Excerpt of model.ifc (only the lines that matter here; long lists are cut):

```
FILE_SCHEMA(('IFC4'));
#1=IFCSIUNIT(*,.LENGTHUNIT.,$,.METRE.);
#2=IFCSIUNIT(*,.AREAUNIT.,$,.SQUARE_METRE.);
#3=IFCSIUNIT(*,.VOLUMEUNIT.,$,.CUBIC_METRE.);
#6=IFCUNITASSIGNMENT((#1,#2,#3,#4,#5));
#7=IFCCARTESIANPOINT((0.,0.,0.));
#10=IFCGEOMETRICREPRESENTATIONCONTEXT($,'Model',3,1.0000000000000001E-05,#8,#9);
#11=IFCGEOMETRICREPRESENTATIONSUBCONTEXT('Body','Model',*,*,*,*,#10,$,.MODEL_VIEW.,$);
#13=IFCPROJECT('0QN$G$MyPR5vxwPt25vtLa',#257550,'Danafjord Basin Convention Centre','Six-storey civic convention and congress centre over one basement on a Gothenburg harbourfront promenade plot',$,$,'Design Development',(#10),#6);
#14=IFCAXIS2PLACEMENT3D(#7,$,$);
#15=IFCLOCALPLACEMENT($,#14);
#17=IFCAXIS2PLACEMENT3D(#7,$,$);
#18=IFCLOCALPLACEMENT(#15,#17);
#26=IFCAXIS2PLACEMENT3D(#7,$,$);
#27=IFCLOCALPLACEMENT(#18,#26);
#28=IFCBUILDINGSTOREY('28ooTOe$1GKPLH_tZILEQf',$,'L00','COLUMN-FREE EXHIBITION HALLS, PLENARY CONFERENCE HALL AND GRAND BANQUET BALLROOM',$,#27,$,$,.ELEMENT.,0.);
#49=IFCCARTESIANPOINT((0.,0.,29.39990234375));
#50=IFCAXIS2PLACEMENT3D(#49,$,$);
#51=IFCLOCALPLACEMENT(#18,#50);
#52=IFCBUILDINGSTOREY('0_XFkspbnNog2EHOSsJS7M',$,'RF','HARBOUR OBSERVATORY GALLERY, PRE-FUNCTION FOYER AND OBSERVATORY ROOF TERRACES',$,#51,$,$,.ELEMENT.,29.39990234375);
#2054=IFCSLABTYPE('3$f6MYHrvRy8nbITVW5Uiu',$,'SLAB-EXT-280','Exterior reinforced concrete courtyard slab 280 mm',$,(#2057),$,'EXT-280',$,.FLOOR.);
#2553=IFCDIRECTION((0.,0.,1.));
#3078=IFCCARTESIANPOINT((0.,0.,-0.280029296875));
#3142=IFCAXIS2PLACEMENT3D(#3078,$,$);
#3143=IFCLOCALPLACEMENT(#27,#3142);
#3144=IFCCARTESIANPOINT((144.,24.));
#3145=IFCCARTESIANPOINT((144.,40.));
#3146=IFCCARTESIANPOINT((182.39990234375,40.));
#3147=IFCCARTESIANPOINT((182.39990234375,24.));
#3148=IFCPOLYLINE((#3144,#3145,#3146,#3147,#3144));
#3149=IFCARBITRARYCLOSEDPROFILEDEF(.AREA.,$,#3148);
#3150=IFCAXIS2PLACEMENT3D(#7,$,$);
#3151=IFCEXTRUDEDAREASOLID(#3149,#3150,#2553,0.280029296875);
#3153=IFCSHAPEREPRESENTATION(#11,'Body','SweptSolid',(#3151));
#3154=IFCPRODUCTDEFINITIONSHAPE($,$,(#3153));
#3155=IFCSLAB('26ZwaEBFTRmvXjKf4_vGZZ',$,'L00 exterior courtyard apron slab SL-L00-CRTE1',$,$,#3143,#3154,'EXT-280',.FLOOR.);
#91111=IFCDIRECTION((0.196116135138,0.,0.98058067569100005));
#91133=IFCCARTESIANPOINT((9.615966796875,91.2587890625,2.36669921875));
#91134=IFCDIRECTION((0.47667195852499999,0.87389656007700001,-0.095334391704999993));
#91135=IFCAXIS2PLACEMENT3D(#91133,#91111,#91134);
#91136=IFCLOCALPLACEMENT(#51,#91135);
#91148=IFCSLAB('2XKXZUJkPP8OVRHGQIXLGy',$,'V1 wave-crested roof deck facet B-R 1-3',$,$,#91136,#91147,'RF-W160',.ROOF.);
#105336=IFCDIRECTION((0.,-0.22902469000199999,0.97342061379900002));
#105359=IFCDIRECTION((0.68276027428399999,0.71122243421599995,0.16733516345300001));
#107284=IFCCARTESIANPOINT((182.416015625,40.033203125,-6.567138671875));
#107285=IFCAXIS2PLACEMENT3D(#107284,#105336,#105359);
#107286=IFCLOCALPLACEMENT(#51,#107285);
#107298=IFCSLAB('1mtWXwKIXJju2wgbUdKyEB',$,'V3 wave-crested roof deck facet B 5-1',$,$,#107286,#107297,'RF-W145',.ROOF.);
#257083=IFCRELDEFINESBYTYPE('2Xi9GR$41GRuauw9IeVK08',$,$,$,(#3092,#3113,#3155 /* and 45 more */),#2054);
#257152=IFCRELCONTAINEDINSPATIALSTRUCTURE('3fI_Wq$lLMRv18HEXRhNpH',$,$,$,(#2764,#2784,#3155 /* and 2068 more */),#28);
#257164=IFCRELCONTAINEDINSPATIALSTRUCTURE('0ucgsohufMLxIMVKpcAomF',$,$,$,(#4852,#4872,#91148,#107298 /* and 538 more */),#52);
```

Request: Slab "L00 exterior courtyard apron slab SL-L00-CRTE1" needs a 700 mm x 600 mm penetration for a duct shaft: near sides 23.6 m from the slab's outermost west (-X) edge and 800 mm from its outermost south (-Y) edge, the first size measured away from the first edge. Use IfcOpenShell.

```python
import numpy as np
import ifcopenshell
import ifcopenshell.api.feature
import ifcopenshell.api.geometry
import ifcopenshell.api.root
import ifcopenshell.geom
import ifcopenshell.util.placement
import ifcopenshell.util.representation
import ifcopenshell.util.shape
import ifcopenshell.util.unit

model = ifcopenshell.open("model.ifc")
unit_scale = ifcopenshell.util.unit.calculate_unit_scale(model)
settings = ifcopenshell.geom.settings()


def volume(element):
    """Net volume in cubic metres, openings subtracted."""
    shape = ifcopenshell.geom.create_shape(settings, element)
    return ifcopenshell.util.shape.get_volume(shape.geometry)


slab = model.by_id(3155)
before = volume(slab)

# Extent in the slab's own axes, in metres. The edges named are its -X and -Y sides.
slab_shape = ifcopenshell.geom.create_shape(settings, slab)
vertices = ifcopenshell.util.shape.get_vertices(slab_shape.geometry)
x_min, y_min, bottom = vertices.min(axis=0)
top = vertices[:, 2].max()

opening = ifcopenshell.api.root.create_entity(model, ifc_class="IfcOpeningElement", name="Duct shaft opening", predefined_type="OPENING")
context = ifcopenshell.util.representation.get_context(model, "Model", "Body", "MODEL_VIEW")
width, depth = 0.7, 0.6
outline = [(0.0, 0.0), (width, 0.0), (width, depth), (0.0, depth), (0.0, 0.0)]
# Overshoot both faces by 50 mm so the cut is clean.
shape = ifcopenshell.api.geometry.add_slab_representation(
    model, context=context, depth=top - bottom + 0.1, polyline=outline
)
ifcopenshell.api.geometry.assign_representation(model, product=opening, representation=shape)

matrix = ifcopenshell.util.placement.get_local_placement(slab.ObjectPlacement)
matrix[:, 3] = matrix @ np.append(np.array([x_min + 23.6, y_min + 0.8, bottom - 0.05]) / unit_scale, 1.0)
ifcopenshell.api.geometry.edit_object_placement(model, product=opening, matrix=matrix, is_si=False)
ifcopenshell.api.feature.add_feature(model, feature=opening, element=slab)

after = volume(slab)

print(f"slab volume {before:.3f} -> {after:.3f} m3")

model.write("model_v2.ifc")
```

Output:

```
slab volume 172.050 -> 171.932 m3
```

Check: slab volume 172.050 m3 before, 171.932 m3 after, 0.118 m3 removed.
